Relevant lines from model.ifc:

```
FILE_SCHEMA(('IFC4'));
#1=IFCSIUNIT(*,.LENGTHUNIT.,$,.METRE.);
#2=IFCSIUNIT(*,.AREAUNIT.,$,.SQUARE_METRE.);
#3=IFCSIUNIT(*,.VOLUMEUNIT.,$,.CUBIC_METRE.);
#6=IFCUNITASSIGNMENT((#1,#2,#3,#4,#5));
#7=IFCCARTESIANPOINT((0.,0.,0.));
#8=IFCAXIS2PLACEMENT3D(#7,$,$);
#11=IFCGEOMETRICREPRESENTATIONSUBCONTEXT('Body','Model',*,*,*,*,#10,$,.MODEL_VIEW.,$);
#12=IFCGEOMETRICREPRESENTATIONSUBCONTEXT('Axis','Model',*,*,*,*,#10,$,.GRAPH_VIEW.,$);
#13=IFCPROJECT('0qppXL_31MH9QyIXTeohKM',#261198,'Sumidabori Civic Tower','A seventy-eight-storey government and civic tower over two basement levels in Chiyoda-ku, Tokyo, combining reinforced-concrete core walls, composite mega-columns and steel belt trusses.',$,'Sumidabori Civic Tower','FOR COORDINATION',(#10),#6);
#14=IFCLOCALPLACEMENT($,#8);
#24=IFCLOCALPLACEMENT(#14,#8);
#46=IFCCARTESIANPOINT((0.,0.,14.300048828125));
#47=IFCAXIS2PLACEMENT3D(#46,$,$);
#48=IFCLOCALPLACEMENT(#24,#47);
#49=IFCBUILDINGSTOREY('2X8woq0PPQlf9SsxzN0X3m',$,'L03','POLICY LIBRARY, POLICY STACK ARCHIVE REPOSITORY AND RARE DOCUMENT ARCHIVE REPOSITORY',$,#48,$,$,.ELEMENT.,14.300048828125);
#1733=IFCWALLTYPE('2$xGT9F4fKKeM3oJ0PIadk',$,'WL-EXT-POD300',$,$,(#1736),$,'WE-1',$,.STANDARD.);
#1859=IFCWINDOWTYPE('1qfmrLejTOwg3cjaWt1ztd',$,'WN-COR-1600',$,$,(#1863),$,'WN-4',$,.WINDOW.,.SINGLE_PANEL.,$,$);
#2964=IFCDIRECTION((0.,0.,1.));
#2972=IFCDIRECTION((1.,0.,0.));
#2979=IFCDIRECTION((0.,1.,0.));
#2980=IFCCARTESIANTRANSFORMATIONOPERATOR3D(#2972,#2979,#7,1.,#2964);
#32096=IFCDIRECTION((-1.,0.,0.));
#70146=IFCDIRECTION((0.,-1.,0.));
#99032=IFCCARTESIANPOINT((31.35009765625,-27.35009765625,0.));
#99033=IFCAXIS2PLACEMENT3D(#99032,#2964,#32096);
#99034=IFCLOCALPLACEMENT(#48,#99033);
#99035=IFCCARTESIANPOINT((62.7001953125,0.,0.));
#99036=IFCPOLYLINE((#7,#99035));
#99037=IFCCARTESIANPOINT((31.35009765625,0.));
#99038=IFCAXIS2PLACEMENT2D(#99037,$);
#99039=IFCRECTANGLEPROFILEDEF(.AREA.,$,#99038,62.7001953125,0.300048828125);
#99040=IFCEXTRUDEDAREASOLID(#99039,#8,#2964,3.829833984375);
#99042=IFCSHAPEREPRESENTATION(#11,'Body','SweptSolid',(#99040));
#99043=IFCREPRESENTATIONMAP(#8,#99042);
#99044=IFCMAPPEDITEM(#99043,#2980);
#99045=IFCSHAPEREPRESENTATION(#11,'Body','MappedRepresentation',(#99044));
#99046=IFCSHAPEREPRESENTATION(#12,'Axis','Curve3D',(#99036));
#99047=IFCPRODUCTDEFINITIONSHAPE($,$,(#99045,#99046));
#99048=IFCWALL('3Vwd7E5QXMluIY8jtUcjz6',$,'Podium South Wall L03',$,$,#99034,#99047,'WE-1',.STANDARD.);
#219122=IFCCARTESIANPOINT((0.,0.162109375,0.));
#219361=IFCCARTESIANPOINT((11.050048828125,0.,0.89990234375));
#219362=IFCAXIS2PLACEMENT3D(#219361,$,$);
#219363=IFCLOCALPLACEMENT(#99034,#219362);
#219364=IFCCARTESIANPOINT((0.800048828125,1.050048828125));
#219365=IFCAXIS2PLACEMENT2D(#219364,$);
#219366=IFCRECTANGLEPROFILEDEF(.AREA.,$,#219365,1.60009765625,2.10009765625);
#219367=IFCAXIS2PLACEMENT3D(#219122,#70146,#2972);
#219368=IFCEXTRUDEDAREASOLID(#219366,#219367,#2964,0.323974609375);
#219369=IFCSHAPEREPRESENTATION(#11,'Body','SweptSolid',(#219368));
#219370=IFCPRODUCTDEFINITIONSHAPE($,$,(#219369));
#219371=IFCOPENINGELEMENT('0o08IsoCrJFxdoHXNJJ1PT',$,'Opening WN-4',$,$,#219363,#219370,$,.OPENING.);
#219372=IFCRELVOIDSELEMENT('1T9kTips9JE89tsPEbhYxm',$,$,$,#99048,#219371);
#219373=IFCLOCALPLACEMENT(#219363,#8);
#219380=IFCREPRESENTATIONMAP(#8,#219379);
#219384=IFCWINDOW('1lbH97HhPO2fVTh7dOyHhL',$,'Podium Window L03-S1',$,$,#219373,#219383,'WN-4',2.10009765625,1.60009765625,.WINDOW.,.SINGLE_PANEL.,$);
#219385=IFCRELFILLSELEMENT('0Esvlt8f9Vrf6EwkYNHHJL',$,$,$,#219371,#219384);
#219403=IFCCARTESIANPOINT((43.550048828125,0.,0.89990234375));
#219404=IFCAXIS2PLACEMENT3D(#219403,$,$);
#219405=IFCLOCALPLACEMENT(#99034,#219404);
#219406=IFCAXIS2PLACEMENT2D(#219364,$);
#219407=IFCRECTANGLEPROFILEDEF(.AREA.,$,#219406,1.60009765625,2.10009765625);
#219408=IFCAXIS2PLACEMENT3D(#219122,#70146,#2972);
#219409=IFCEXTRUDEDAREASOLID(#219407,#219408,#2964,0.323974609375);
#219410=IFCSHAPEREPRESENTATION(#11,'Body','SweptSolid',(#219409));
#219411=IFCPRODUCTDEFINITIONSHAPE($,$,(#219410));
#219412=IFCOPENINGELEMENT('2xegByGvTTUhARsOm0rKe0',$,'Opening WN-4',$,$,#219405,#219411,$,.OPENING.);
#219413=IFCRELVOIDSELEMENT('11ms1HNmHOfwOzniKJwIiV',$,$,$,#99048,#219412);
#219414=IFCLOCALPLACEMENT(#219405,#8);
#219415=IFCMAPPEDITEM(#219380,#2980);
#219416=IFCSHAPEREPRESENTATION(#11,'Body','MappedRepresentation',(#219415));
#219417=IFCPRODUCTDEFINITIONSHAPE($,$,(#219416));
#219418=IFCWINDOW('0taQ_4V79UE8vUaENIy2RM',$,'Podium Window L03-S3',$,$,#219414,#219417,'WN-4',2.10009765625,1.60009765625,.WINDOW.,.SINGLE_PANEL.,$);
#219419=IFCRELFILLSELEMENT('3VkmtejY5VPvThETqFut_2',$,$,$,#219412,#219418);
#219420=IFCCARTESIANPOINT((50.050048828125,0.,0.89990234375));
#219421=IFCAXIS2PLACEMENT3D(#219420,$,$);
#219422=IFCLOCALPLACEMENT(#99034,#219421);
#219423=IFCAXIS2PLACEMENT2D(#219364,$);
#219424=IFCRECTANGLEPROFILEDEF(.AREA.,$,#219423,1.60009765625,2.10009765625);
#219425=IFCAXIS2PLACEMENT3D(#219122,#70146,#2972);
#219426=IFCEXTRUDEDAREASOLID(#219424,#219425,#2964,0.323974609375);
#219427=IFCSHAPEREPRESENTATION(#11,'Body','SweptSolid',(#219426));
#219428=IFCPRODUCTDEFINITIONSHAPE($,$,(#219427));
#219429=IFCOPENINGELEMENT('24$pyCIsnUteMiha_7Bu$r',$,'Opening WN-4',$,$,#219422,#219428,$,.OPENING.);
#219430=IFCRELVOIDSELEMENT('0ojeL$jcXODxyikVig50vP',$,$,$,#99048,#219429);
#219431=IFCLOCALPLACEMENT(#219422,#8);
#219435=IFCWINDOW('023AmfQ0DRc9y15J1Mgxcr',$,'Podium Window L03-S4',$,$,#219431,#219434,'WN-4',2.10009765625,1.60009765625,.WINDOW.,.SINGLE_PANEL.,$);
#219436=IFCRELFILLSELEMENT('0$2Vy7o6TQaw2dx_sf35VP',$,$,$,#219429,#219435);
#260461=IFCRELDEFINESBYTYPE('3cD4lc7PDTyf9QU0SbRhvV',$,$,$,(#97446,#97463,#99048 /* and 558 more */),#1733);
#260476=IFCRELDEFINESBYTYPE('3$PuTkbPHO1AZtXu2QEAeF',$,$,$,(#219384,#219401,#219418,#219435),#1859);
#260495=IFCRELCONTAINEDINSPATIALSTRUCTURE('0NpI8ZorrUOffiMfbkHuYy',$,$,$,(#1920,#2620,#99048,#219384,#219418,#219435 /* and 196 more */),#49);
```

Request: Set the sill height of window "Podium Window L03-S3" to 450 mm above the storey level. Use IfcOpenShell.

```python
import numpy as np
import ifcopenshell
import ifcopenshell.api.geometry
import ifcopenshell.geom
import ifcopenshell.util.element
import ifcopenshell.util.placement
import ifcopenshell.util.shape
import ifcopenshell.util.unit

model = ifcopenshell.open("model.ifc")
unit_scale = ifcopenshell.util.unit.calculate_unit_scale(model)

window = model.by_guid("0taQ_4V79UE8vUaENIy2RM")
opening = window.FillsVoids[0].RelatingOpeningElement
storey = ifcopenshell.util.element.get_container(window, ifc_class="IfcBuildingStorey")
level = ifcopenshell.util.placement.get_local_placement(storey.ObjectPlacement)[2, 3]

# The opening's origin need not be at the sill, so measure its lowest point.
shape = ifcopenshell.geom.create_shape(ifcopenshell.geom.settings(), opening)
bottom = ifcopenshell.util.shape.get_shape_bottom_elevation(shape, shape.geometry) / unit_scale
dz = level + 0.45 / unit_scale - bottom

shift = np.array([0.0, 0.0, dz])
# The window is placed relative to its opening, so it follows when the opening moves.
matrix = ifcopenshell.util.placement.get_local_placement(opening.ObjectPlacement)
matrix[:3, 3] += shift
ifcopenshell.api.geometry.edit_object_placement(
    model, product=opening, matrix=matrix, is_si=False, should_transform_children=True
)

print(f"moved by {dz * unit_scale:+.3f} m")

model.write("model_rev.ifc")
```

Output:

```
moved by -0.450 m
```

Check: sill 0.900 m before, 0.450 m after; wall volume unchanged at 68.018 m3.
